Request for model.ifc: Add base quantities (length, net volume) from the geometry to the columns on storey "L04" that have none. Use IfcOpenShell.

First a look at what the model holds.

```python
import ifcopenshell
import ifcopenshell.util.element
import ifcopenshell.util.unit

model = ifcopenshell.open("model.ifc")
print(model.schema)
for unit_type in ("LENGTHUNIT", "AREAUNIT", "VOLUMEUNIT"):
    print(unit_type, ifcopenshell.util.unit.calculate_unit_scale(model, unit_type))
storey = next(s for s in model.by_type("IfcBuildingStorey") if s.Name == "L04")
columns = [e for e in ifcopenshell.util.element.get_decomposition(storey) if e.is_a("IfcColumn")]
for e in sorted(columns, key=lambda e: e.id()):
    print(e.id(), e.is_a(), e.Name, list(ifcopenshell.util.element.get_psets(e, qtos_only=True)), sep=" | ")
```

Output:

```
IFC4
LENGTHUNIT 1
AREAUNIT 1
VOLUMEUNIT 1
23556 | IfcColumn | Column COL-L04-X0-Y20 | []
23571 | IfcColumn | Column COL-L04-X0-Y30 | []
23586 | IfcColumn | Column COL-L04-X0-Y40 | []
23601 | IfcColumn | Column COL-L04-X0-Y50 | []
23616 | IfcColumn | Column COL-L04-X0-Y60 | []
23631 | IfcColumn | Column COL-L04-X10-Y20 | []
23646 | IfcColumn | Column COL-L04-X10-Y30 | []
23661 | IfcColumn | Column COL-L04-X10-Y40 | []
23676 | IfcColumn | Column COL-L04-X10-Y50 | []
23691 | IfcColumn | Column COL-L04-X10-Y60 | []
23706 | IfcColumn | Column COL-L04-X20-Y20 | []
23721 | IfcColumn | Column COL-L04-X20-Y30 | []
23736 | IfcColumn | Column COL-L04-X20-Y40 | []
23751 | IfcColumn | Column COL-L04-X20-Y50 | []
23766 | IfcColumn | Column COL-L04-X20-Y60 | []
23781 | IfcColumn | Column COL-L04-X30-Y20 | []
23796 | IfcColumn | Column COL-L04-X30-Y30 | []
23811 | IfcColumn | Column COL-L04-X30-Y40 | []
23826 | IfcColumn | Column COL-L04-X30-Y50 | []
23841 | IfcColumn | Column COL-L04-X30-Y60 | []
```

```python
import ifcopenshell
import ifcopenshell.api.pset
import ifcopenshell.geom
import ifcopenshell.util.element
import ifcopenshell.util.shape
import ifcopenshell.util.unit

model = ifcopenshell.open("model.ifc")
unit_scale = ifcopenshell.util.unit.calculate_unit_scale(model)
volume_scale = ifcopenshell.util.unit.calculate_unit_scale(model, "VOLUMEUNIT")
settings = ifcopenshell.geom.settings()

storey = next(s for s in model.by_type("IfcBuildingStorey") if s.Name == "L04")
columns = [e for e in ifcopenshell.util.element.get_decomposition(storey) if e.is_a("IfcColumn")]

for e in sorted(columns, key=lambda e: e.id()):
    if ifcopenshell.util.element.get_psets(e, qtos_only=True, should_inherit=False):
        continue
    # Geometry comes back in metres, in the element's own axes.
    shape = ifcopenshell.geom.create_shape(settings, e)
    values = {
        "Length": ifcopenshell.util.shape.get_z(shape.geometry) / unit_scale,
        "NetVolume": ifcopenshell.util.shape.get_volume(shape.geometry) / volume_scale,
    }
    qto = ifcopenshell.api.pset.add_qto(model, product=e, name="Qto_ColumnBaseQuantities")
    ifcopenshell.api.pset.edit_qto(model, qto=qto, properties=values)
    print(e.id(), {k: round(v, 3) for k, v in values.items()})

model.write("model_v2.ifc")
```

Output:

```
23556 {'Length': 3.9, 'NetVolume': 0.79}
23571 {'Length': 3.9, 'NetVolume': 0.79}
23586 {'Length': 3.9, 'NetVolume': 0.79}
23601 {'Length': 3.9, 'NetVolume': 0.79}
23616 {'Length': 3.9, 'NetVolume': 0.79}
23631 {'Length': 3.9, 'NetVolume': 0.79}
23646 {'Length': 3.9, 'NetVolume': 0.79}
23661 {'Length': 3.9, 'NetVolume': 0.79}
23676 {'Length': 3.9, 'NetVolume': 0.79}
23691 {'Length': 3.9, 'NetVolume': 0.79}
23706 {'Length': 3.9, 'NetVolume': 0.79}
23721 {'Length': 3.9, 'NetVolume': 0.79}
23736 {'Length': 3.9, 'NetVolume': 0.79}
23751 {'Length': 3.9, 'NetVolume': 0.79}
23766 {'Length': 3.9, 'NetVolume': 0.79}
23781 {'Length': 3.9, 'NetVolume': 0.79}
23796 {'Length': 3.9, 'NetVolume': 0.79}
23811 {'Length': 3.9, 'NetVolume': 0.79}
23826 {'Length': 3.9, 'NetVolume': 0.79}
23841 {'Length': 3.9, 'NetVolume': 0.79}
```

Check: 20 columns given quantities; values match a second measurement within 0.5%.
